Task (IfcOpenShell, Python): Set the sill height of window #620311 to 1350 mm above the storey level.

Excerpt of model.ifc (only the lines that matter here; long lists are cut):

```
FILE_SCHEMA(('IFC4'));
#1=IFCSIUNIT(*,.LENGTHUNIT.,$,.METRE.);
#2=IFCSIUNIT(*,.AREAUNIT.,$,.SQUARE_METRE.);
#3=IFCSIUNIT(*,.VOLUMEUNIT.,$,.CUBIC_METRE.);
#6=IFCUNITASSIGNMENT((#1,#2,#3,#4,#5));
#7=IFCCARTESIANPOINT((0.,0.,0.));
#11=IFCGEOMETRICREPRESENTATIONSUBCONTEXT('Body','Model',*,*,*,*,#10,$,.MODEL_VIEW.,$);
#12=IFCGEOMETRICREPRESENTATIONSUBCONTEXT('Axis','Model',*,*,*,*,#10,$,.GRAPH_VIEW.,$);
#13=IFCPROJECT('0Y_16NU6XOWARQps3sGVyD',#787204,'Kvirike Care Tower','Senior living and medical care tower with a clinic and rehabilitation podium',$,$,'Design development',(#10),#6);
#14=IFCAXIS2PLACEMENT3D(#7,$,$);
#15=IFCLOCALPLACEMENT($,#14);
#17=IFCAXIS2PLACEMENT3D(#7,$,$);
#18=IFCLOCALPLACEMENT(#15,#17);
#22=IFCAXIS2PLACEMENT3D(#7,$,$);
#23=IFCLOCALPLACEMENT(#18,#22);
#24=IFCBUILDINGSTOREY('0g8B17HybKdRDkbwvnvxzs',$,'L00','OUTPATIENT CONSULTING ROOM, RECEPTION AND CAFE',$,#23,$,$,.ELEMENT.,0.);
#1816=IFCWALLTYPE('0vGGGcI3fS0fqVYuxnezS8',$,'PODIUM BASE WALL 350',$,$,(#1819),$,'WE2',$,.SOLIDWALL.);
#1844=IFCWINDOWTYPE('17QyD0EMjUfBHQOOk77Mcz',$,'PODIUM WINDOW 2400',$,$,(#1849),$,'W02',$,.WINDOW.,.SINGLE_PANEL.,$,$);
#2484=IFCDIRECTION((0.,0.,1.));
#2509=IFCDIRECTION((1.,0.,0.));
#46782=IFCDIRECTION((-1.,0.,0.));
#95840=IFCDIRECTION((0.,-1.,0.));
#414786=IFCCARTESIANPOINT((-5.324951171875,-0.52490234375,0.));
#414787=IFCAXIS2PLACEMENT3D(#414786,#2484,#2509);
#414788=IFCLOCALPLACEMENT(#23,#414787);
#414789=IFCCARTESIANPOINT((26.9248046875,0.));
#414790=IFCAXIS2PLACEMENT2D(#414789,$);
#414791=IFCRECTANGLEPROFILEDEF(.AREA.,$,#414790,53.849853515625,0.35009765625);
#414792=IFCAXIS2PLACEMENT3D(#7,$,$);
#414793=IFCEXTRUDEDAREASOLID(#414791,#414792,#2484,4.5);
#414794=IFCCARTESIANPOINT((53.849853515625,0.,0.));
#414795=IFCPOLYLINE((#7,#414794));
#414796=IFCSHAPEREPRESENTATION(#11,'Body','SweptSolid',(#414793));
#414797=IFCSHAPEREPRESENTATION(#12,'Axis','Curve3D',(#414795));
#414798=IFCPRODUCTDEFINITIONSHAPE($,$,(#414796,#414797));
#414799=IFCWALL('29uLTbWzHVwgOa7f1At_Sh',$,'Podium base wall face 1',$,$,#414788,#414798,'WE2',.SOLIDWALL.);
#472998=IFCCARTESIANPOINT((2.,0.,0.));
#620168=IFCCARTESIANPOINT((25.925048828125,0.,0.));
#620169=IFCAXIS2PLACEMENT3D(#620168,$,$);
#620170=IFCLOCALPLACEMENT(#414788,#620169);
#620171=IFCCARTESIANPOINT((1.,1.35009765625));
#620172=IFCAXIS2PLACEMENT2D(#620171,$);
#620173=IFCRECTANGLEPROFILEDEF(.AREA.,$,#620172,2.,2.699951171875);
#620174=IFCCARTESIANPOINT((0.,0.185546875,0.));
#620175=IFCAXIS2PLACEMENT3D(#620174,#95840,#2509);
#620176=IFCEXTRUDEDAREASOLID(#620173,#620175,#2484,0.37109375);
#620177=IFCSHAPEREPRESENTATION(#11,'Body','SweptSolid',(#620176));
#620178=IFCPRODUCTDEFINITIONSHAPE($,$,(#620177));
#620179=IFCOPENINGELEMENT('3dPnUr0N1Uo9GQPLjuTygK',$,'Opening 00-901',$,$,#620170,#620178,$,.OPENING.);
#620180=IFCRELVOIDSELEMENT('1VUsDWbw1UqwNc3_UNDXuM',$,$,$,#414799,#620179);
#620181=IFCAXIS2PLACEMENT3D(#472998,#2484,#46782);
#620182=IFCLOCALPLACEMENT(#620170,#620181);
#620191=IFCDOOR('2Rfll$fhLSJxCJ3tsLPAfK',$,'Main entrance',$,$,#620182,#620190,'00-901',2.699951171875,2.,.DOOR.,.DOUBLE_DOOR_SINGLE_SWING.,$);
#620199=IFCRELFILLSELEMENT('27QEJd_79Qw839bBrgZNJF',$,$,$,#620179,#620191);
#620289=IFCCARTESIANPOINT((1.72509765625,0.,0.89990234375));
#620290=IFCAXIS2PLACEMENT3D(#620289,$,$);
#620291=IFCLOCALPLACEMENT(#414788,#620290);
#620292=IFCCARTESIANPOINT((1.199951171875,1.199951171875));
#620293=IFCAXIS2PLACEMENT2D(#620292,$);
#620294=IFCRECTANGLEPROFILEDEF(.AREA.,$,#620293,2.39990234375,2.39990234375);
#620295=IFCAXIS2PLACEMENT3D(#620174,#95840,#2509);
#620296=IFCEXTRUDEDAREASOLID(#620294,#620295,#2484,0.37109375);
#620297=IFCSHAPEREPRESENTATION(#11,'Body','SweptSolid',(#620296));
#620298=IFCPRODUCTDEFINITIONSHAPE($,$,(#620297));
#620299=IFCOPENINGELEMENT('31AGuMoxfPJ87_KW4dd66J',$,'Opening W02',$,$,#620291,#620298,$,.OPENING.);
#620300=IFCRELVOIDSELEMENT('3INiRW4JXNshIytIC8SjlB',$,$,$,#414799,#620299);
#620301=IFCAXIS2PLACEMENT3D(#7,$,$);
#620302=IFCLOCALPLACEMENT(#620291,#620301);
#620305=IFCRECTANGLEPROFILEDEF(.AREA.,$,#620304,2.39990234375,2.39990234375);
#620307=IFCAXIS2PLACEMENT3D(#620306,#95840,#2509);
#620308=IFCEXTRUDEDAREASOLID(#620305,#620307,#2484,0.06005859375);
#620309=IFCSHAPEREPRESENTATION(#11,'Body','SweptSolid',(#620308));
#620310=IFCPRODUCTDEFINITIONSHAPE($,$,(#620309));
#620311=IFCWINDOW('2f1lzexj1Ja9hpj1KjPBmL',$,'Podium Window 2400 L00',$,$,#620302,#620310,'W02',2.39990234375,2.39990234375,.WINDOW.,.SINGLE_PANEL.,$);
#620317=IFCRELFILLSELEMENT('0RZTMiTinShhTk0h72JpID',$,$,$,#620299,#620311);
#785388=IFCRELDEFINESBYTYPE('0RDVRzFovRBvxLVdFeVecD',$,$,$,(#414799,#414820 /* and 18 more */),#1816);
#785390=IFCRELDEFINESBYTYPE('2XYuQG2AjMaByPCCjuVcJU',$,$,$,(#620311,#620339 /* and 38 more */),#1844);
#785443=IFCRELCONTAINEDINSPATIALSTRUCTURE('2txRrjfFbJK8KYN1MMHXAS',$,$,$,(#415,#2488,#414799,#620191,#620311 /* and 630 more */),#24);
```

```python
import numpy as np
import ifcopenshell
import ifcopenshell.api.geometry
import ifcopenshell.geom
import ifcopenshell.util.element
import ifcopenshell.util.placement
import ifcopenshell.util.shape
import ifcopenshell.util.unit

model = ifcopenshell.open("model.ifc")
unit_scale = ifcopenshell.util.unit.calculate_unit_scale(model)

window = model.by_id(620311)
opening = window.FillsVoids[0].RelatingOpeningElement
storey = ifcopenshell.util.element.get_container(window, ifc_class="IfcBuildingStorey")
level = ifcopenshell.util.placement.get_local_placement(storey.ObjectPlacement)[2, 3]

# The opening's origin need not be at the sill, so measure its lowest point.
shape = ifcopenshell.geom.create_shape(ifcopenshell.geom.settings(), opening)
bottom = ifcopenshell.util.shape.get_shape_bottom_elevation(shape, shape.geometry) / unit_scale
dz = level + 1.35 / unit_scale - bottom

shift = np.array([0.0, 0.0, dz])
# The window is placed relative to its opening, so it follows when the opening moves.
matrix = ifcopenshell.util.placement.get_local_placement(opening.ObjectPlacement)
matrix[:3, 3] += shift
ifcopenshell.api.geometry.edit_object_placement(
    model, product=opening, matrix=matrix, is_si=False, should_transform_children=True
)

print(f"moved by {dz * unit_scale:+.3f} m")

model.write("model_updated.ifc")
```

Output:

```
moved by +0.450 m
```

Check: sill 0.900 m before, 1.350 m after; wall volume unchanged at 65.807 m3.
